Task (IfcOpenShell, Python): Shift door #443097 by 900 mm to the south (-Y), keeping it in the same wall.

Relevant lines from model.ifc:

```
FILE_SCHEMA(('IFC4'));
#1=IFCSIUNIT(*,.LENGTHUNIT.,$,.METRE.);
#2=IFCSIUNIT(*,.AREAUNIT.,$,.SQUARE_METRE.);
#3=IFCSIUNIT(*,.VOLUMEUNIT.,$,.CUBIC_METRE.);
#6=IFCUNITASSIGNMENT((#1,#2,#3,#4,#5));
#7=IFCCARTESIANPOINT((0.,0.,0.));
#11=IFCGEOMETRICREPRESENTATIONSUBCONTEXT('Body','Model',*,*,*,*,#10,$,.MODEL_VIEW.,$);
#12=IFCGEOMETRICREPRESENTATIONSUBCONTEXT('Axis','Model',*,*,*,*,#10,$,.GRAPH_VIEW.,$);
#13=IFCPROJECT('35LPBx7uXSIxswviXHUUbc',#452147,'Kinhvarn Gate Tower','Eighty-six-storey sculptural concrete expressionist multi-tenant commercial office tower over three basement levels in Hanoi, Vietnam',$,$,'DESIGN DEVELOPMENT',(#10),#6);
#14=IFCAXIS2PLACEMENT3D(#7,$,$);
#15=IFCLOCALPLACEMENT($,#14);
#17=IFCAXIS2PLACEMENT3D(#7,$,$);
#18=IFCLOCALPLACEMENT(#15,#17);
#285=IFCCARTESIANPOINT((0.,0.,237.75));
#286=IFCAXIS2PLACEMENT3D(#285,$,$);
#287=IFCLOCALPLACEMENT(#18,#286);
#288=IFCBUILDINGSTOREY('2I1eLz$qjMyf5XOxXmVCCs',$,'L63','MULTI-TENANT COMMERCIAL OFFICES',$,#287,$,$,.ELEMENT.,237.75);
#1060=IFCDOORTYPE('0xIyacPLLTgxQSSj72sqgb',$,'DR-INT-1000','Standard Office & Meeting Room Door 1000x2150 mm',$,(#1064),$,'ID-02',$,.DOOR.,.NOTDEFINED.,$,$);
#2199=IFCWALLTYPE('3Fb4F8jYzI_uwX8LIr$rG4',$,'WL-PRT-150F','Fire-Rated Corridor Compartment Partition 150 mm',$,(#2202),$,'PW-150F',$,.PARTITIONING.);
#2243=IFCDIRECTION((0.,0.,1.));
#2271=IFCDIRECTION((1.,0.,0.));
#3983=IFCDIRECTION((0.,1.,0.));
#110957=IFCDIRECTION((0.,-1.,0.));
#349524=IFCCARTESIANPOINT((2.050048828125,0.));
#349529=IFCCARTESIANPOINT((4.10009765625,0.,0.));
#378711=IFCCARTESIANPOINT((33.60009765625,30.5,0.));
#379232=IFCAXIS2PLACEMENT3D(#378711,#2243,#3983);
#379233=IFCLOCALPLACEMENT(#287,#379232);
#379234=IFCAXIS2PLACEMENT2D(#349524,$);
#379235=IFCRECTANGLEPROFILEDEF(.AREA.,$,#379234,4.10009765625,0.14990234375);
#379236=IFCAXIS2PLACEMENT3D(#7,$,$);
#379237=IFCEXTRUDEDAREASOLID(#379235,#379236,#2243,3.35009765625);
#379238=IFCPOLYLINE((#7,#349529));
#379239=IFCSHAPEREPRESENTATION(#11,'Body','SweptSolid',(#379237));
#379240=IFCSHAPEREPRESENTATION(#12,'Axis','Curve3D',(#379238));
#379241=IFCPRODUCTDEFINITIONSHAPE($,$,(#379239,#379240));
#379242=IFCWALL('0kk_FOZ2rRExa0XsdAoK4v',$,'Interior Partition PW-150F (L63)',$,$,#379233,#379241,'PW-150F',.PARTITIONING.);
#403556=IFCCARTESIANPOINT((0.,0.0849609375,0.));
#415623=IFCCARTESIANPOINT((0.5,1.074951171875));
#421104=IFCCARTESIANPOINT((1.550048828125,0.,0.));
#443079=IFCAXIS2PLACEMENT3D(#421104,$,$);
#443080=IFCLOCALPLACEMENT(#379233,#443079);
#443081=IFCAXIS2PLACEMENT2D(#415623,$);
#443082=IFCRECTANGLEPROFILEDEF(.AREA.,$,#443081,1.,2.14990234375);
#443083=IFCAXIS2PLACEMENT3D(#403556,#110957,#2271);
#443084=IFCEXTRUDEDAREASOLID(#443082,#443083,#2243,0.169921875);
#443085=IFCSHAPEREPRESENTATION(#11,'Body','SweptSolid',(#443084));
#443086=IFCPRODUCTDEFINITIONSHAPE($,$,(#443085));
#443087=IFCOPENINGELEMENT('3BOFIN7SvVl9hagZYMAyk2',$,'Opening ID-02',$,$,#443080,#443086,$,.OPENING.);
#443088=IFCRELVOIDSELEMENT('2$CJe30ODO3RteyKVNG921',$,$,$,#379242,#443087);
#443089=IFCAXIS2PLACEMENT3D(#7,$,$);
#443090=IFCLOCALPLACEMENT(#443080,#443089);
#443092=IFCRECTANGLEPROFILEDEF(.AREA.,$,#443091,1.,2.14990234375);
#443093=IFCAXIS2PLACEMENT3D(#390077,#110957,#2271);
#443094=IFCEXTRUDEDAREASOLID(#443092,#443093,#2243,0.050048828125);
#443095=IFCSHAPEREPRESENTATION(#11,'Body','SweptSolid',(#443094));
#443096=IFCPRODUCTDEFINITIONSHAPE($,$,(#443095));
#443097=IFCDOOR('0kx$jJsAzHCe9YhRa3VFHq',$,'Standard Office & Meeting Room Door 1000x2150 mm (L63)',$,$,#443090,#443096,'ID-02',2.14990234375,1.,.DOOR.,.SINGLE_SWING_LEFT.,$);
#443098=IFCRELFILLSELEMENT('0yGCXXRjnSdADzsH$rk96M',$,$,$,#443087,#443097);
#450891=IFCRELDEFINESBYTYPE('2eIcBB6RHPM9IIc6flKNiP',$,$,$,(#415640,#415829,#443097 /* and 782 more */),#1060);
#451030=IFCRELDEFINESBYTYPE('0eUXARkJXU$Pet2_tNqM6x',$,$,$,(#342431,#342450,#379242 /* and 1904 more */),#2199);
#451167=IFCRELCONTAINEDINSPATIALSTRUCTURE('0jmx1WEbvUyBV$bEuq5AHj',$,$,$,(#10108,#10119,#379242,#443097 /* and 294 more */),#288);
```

```python
import ifcopenshell
import ifcopenshell.api.geometry
import ifcopenshell.util.placement
import ifcopenshell.util.unit

model = ifcopenshell.open("model.ifc")
unit_scale = ifcopenshell.util.unit.calculate_unit_scale(model)

door = model.by_guid("0kx$jJsAzHCe9YhRa3VFHq")
opening = door.FillsVoids[0].RelatingOpeningElement
wall = opening.VoidsElements[0].RelatingBuildingElement

wall_matrix = ifcopenshell.util.placement.get_local_placement(wall.ObjectPlacement)
shift = wall_matrix[:3, 0] * -0.9 / unit_scale
before = ifcopenshell.util.placement.get_local_placement(door.ObjectPlacement)[:3, 3].copy()

# The door is placed relative to its opening, so it follows when the opening moves.
matrix = ifcopenshell.util.placement.get_local_placement(opening.ObjectPlacement)
matrix[:3, 3] += shift
ifcopenshell.api.geometry.edit_object_placement(
    model, product=opening, matrix=matrix, is_si=False, should_transform_children=True
)

after = ifcopenshell.util.placement.get_local_placement(door.ObjectPlacement)[:3, 3]
print("door moved by", (after - before).round(3) + 0.0)

model.write("model_v2.ifc")
```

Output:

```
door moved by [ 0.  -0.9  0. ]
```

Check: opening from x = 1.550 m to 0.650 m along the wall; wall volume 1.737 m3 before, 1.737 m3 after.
